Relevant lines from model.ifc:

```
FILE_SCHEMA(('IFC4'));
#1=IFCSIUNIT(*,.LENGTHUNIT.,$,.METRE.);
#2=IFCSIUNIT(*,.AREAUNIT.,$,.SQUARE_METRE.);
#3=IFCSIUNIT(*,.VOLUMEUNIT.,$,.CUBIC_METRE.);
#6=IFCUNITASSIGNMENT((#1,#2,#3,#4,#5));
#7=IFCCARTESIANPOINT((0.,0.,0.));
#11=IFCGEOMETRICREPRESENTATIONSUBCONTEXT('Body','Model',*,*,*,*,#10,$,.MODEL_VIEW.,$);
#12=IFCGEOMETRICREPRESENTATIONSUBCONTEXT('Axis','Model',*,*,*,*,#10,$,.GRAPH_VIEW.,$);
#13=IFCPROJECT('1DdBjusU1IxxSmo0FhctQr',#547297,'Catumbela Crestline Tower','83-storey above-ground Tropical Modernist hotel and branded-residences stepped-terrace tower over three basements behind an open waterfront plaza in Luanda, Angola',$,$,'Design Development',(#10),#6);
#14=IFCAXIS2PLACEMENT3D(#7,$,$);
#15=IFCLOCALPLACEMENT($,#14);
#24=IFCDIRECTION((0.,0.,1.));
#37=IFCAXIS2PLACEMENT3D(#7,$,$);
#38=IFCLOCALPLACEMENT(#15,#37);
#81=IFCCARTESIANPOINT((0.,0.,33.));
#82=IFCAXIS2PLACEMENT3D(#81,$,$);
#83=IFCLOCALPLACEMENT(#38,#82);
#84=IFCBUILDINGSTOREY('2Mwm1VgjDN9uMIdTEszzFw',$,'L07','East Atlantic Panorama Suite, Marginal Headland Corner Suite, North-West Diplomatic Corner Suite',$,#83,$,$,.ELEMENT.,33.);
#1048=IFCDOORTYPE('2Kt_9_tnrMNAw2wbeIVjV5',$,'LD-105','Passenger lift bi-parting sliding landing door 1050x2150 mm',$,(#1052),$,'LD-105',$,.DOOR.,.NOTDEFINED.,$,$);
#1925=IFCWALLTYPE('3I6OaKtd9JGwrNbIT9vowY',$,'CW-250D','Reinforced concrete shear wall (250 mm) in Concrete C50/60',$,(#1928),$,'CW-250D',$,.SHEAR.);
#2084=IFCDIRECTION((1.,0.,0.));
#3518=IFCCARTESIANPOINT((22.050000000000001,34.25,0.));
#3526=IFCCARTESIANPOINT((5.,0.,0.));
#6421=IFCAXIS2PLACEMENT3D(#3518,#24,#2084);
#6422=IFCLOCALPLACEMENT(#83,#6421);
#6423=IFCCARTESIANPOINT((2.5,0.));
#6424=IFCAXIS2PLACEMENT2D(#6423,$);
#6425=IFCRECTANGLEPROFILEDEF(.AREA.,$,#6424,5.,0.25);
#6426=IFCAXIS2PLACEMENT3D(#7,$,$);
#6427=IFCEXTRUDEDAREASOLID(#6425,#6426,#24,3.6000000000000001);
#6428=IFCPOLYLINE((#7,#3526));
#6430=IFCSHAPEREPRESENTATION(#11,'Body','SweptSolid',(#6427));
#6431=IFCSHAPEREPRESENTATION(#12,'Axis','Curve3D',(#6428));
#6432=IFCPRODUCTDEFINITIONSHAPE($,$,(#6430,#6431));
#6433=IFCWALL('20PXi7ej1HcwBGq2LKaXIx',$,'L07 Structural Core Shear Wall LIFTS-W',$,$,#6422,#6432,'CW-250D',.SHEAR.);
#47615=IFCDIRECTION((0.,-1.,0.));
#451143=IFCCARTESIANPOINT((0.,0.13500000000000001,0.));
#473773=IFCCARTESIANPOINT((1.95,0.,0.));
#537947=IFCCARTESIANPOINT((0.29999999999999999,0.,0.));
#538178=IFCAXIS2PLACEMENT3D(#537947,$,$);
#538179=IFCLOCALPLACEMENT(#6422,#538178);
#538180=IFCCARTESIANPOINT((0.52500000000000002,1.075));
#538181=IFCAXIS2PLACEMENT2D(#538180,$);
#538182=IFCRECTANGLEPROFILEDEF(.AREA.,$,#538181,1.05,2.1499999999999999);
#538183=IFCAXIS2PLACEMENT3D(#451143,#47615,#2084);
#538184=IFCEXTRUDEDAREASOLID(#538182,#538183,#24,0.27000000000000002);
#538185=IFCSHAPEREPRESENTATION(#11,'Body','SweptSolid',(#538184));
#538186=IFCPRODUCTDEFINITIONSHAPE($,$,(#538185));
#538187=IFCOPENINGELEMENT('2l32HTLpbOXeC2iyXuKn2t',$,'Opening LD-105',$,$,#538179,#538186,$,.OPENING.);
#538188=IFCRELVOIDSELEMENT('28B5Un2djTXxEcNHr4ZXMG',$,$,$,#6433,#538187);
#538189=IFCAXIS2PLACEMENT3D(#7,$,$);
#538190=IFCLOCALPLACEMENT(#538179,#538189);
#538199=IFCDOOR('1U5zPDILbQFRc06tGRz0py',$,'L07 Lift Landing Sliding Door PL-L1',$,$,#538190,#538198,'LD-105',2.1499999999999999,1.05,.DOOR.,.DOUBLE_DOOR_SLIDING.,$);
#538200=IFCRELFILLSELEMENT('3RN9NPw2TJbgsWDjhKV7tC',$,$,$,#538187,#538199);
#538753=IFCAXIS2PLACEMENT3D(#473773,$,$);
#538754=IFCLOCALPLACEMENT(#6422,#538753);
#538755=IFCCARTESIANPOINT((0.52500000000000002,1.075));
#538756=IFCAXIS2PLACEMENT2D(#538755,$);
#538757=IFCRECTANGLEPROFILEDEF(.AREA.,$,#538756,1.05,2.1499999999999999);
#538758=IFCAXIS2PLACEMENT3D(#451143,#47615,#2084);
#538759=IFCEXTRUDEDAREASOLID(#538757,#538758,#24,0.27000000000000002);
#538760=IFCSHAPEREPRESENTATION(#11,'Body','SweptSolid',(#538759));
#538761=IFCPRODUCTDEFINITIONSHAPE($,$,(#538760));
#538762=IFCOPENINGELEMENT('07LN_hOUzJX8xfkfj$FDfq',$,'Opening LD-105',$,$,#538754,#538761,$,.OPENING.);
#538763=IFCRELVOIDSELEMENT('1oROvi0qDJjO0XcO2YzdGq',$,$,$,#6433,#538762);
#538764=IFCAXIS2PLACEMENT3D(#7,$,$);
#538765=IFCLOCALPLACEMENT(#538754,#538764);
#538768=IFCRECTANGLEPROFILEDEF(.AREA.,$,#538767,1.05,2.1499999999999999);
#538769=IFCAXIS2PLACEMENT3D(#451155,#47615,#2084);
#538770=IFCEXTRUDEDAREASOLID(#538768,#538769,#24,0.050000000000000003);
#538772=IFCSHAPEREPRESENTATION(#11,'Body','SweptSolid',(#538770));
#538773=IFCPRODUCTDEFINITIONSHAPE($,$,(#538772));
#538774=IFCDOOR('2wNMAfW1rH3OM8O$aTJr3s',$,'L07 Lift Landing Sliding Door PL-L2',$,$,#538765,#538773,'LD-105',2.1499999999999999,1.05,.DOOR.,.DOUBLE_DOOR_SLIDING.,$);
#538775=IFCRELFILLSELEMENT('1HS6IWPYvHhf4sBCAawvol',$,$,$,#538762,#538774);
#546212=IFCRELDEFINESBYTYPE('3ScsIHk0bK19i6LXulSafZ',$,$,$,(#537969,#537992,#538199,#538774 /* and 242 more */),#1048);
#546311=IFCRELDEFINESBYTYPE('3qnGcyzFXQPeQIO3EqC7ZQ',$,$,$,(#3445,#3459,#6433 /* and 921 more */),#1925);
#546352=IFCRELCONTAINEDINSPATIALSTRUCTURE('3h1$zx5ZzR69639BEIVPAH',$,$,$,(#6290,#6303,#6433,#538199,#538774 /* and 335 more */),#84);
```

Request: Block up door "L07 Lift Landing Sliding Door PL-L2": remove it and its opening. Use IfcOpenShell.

```python
import ifcopenshell
import ifcopenshell.api.feature
import ifcopenshell.api.root
import ifcopenshell.geom
import ifcopenshell.util.shape

model = ifcopenshell.open("model.ifc")
settings = ifcopenshell.geom.settings()


def volume(element):
    """Net volume in cubic metres, openings subtracted."""
    shape = ifcopenshell.geom.create_shape(settings, element)
    return ifcopenshell.util.shape.get_volume(shape.geometry)


door = model.by_id(538774)
opening = door.FillsVoids[0].RelatingOpeningElement
wall = opening.VoidsElements[0].RelatingBuildingElement
before = volume(wall)

ifcopenshell.api.root.remove_product(model, product=door)
ifcopenshell.api.feature.remove_feature(model, feature=opening)

after = volume(wall)

print(f"wall volume {before:.3f} -> {after:.3f} m3")

model.write("model_v2.ifc")
```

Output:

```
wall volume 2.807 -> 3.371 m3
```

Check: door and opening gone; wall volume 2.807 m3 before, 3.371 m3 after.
